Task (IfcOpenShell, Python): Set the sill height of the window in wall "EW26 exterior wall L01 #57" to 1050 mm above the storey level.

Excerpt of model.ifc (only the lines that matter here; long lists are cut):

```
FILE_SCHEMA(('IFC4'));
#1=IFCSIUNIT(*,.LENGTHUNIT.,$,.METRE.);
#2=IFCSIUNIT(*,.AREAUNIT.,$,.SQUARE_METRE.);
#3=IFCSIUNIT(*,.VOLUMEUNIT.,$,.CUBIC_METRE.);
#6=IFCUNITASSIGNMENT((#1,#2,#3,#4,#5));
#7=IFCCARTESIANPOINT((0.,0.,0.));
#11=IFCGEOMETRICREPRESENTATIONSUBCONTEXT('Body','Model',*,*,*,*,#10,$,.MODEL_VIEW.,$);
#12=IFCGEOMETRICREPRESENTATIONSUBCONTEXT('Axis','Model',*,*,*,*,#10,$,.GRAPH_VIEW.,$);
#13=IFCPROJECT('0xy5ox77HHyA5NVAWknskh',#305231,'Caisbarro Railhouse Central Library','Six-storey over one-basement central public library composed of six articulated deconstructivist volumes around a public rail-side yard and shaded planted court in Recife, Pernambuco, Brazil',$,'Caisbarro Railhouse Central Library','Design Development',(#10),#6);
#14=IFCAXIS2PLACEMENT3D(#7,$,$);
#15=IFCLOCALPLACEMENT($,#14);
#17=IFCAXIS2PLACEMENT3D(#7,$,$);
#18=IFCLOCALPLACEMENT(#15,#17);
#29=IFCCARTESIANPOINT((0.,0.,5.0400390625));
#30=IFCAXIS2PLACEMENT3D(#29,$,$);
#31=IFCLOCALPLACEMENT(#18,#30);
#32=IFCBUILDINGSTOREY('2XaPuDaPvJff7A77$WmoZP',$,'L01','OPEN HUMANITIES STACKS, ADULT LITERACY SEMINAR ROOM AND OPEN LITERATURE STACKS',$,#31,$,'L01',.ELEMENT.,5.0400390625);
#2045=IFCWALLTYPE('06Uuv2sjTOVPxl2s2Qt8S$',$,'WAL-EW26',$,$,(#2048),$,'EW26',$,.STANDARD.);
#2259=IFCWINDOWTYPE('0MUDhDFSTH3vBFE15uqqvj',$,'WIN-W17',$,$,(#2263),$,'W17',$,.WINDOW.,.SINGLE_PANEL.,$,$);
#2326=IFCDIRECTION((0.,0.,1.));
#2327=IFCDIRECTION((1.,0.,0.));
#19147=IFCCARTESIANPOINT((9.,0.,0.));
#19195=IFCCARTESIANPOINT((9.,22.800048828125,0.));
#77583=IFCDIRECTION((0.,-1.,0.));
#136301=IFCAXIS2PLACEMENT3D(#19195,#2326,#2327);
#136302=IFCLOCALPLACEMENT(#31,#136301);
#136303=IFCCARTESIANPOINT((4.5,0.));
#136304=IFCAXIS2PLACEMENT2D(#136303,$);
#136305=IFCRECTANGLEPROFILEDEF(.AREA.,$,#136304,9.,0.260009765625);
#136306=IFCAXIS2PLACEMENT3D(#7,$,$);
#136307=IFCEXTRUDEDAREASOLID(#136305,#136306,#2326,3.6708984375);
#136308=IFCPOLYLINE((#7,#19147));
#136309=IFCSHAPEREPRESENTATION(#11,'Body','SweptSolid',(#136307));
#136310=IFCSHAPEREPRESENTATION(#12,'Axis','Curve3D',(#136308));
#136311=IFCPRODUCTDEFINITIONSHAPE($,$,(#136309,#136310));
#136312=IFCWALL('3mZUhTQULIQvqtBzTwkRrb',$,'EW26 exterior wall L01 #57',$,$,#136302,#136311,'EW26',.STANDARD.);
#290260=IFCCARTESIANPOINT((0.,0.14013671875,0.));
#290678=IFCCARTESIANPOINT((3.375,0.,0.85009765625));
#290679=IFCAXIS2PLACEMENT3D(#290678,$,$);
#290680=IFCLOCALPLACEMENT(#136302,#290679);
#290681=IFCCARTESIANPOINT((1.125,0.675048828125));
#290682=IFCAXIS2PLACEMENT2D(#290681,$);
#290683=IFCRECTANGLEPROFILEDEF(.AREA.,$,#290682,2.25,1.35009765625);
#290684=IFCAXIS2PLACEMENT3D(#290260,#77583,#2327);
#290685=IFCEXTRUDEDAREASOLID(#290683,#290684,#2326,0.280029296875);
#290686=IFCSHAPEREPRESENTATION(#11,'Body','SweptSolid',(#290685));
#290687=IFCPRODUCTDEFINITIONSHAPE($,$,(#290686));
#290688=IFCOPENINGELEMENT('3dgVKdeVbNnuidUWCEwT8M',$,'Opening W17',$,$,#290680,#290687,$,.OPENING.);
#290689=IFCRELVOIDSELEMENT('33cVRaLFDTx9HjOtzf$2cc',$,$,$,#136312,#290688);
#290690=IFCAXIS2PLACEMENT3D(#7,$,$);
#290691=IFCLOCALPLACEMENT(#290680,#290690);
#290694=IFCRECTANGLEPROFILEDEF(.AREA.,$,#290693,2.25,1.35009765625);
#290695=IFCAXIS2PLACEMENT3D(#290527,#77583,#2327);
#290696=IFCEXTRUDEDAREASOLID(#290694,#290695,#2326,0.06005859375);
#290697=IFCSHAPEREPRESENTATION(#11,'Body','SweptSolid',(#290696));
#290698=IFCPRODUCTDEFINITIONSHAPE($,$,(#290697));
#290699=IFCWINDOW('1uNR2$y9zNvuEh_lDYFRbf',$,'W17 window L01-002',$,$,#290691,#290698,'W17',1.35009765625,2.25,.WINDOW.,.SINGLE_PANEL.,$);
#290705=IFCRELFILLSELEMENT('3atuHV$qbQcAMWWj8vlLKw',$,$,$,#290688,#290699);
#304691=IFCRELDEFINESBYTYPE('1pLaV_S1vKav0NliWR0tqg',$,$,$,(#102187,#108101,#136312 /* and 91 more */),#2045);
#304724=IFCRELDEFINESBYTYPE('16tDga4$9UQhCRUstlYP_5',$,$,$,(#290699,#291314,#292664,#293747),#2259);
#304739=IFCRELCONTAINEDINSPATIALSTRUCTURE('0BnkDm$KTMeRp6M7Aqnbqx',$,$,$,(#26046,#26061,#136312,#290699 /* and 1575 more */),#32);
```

```python
import numpy as np
import ifcopenshell
import ifcopenshell.api.geometry
import ifcopenshell.geom
import ifcopenshell.util.element
import ifcopenshell.util.placement
import ifcopenshell.util.shape
import ifcopenshell.util.unit

model = ifcopenshell.open("model.ifc")
unit_scale = ifcopenshell.util.unit.calculate_unit_scale(model)

window = model.by_guid("1uNR2$y9zNvuEh_lDYFRbf")
opening = window.FillsVoids[0].RelatingOpeningElement
storey = ifcopenshell.util.element.get_container(window, ifc_class="IfcBuildingStorey")
level = ifcopenshell.util.placement.get_local_placement(storey.ObjectPlacement)[2, 3]

# The opening's origin need not be at the sill, so measure its lowest point.
shape = ifcopenshell.geom.create_shape(ifcopenshell.geom.settings(), opening)
bottom = ifcopenshell.util.shape.get_shape_bottom_elevation(shape, shape.geometry) / unit_scale
dz = level + 1.05 - bottom

shift = np.array([0.0, 0.0, dz])
# The window is placed relative to its opening, so it follows when the opening moves.
matrix = ifcopenshell.util.placement.get_local_placement(opening.ObjectPlacement)
matrix[:3, 3] += shift
ifcopenshell.api.geometry.edit_object_placement(
    model, product=opening, matrix=matrix, is_si=False, should_transform_children=True
)

print(f"moved by {dz * unit_scale:+.3f} m")

model.write("model-out.ifc")
```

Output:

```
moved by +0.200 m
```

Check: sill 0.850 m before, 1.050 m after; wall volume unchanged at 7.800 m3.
